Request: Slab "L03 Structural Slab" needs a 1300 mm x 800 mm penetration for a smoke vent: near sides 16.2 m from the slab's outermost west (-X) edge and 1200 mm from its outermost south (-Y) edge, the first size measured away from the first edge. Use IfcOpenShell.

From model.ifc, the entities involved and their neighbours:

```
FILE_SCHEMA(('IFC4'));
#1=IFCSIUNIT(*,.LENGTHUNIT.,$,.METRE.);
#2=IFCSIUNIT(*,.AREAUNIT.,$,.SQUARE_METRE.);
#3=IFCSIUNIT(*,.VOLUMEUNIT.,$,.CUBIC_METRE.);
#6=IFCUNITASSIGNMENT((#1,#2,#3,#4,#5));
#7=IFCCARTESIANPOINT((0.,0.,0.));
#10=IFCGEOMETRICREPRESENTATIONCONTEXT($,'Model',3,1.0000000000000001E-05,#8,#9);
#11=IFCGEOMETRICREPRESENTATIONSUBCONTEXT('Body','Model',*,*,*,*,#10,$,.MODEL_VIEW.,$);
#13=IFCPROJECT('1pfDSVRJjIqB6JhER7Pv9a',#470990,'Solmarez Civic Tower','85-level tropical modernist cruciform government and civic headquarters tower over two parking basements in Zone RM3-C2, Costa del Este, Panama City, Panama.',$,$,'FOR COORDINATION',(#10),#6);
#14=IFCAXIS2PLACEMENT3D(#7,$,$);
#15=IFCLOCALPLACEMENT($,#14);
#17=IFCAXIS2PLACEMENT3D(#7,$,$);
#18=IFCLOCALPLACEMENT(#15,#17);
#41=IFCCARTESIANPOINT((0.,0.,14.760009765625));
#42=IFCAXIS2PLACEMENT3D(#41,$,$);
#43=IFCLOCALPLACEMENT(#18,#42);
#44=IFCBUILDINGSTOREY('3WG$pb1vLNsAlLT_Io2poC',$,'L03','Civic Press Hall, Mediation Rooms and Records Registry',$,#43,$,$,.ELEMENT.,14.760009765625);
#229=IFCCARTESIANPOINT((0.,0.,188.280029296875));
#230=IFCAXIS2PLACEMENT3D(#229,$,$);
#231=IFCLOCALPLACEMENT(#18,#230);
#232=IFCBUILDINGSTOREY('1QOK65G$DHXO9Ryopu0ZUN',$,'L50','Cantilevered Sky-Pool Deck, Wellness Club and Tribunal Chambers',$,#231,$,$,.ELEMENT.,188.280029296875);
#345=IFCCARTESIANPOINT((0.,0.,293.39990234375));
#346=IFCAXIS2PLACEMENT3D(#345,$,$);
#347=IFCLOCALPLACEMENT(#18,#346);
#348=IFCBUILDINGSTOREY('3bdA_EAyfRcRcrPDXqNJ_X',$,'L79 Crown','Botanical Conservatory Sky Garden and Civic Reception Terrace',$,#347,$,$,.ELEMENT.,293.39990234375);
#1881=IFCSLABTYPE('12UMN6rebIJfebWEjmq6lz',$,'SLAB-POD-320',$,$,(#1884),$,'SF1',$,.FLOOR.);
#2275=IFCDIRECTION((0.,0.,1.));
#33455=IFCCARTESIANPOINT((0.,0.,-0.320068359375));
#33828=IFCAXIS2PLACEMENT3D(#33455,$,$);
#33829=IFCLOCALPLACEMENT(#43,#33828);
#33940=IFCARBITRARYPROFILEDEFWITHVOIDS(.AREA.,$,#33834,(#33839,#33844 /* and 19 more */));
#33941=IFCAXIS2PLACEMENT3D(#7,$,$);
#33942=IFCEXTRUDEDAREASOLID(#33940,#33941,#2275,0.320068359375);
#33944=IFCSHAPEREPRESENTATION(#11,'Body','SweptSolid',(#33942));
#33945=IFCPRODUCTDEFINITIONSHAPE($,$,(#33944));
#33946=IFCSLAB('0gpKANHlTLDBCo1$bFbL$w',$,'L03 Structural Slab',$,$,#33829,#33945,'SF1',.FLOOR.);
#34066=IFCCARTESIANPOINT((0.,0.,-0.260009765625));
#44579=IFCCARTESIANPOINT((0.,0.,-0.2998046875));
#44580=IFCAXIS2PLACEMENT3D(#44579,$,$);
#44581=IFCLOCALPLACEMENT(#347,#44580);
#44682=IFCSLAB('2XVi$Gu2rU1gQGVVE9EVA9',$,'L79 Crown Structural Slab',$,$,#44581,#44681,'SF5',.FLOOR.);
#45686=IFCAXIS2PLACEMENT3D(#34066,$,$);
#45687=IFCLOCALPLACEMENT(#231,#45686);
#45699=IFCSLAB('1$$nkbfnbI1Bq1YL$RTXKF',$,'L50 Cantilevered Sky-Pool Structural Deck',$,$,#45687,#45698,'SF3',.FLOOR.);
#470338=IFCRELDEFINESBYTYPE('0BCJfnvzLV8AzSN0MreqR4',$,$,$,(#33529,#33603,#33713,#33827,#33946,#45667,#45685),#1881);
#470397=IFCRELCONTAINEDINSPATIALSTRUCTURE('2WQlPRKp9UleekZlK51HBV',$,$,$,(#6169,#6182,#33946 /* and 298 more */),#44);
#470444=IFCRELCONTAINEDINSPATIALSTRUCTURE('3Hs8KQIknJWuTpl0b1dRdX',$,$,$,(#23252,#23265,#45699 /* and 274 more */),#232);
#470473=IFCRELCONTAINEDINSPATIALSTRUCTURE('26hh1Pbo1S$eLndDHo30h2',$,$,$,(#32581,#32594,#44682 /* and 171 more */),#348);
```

```python
import numpy as np
import ifcopenshell
import ifcopenshell.api.feature
import ifcopenshell.api.geometry
import ifcopenshell.api.root
import ifcopenshell.geom
import ifcopenshell.util.placement
import ifcopenshell.util.representation
import ifcopenshell.util.shape
import ifcopenshell.util.unit

model = ifcopenshell.open("model.ifc")
unit_scale = ifcopenshell.util.unit.calculate_unit_scale(model)
settings = ifcopenshell.geom.settings()


def volume(element):
    """Net volume in cubic metres, openings subtracted."""
    shape = ifcopenshell.geom.create_shape(settings, element)
    return ifcopenshell.util.shape.get_volume(shape.geometry)


slab = model.by_id(33946)
before = volume(slab)

# Extent in the slab's own axes, in metres. The edges named are its -X and -Y sides.
slab_shape = ifcopenshell.geom.create_shape(settings, slab)
vertices = ifcopenshell.util.shape.get_vertices(slab_shape.geometry)
x_min, y_min, bottom = vertices.min(axis=0)
top = vertices[:, 2].max()

opening = ifcopenshell.api.root.create_entity(model, ifc_class="IfcOpeningElement", name="Smoke vent opening", predefined_type="OPENING")
context = ifcopenshell.util.representation.get_context(model, "Model", "Body", "MODEL_VIEW")
width, depth = 1.3, 0.8
outline = [(0.0, 0.0), (width, 0.0), (width, depth), (0.0, depth), (0.0, 0.0)]
# Overshoot both faces by 50 mm so the cut is clean.
shape = ifcopenshell.api.geometry.add_slab_representation(
    model, context=context, depth=top - bottom + 0.1, polyline=outline
)
ifcopenshell.api.geometry.assign_representation(model, product=opening, representation=shape)

matrix = ifcopenshell.util.placement.get_local_placement(slab.ObjectPlacement)
matrix[:, 3] = matrix @ np.append(np.array([x_min + 16.2, y_min + 1.2, bottom - 0.05]) / unit_scale, 1.0)
ifcopenshell.api.geometry.edit_object_placement(model, product=opening, matrix=matrix, is_si=False)
ifcopenshell.api.feature.add_feature(model, feature=opening, element=slab)

after = volume(slab)

print(f"slab volume {before:.3f} -> {after:.3f} m3")

model.write("model_updated.ifc")
```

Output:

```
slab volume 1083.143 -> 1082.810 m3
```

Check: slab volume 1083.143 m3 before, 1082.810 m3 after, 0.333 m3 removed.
